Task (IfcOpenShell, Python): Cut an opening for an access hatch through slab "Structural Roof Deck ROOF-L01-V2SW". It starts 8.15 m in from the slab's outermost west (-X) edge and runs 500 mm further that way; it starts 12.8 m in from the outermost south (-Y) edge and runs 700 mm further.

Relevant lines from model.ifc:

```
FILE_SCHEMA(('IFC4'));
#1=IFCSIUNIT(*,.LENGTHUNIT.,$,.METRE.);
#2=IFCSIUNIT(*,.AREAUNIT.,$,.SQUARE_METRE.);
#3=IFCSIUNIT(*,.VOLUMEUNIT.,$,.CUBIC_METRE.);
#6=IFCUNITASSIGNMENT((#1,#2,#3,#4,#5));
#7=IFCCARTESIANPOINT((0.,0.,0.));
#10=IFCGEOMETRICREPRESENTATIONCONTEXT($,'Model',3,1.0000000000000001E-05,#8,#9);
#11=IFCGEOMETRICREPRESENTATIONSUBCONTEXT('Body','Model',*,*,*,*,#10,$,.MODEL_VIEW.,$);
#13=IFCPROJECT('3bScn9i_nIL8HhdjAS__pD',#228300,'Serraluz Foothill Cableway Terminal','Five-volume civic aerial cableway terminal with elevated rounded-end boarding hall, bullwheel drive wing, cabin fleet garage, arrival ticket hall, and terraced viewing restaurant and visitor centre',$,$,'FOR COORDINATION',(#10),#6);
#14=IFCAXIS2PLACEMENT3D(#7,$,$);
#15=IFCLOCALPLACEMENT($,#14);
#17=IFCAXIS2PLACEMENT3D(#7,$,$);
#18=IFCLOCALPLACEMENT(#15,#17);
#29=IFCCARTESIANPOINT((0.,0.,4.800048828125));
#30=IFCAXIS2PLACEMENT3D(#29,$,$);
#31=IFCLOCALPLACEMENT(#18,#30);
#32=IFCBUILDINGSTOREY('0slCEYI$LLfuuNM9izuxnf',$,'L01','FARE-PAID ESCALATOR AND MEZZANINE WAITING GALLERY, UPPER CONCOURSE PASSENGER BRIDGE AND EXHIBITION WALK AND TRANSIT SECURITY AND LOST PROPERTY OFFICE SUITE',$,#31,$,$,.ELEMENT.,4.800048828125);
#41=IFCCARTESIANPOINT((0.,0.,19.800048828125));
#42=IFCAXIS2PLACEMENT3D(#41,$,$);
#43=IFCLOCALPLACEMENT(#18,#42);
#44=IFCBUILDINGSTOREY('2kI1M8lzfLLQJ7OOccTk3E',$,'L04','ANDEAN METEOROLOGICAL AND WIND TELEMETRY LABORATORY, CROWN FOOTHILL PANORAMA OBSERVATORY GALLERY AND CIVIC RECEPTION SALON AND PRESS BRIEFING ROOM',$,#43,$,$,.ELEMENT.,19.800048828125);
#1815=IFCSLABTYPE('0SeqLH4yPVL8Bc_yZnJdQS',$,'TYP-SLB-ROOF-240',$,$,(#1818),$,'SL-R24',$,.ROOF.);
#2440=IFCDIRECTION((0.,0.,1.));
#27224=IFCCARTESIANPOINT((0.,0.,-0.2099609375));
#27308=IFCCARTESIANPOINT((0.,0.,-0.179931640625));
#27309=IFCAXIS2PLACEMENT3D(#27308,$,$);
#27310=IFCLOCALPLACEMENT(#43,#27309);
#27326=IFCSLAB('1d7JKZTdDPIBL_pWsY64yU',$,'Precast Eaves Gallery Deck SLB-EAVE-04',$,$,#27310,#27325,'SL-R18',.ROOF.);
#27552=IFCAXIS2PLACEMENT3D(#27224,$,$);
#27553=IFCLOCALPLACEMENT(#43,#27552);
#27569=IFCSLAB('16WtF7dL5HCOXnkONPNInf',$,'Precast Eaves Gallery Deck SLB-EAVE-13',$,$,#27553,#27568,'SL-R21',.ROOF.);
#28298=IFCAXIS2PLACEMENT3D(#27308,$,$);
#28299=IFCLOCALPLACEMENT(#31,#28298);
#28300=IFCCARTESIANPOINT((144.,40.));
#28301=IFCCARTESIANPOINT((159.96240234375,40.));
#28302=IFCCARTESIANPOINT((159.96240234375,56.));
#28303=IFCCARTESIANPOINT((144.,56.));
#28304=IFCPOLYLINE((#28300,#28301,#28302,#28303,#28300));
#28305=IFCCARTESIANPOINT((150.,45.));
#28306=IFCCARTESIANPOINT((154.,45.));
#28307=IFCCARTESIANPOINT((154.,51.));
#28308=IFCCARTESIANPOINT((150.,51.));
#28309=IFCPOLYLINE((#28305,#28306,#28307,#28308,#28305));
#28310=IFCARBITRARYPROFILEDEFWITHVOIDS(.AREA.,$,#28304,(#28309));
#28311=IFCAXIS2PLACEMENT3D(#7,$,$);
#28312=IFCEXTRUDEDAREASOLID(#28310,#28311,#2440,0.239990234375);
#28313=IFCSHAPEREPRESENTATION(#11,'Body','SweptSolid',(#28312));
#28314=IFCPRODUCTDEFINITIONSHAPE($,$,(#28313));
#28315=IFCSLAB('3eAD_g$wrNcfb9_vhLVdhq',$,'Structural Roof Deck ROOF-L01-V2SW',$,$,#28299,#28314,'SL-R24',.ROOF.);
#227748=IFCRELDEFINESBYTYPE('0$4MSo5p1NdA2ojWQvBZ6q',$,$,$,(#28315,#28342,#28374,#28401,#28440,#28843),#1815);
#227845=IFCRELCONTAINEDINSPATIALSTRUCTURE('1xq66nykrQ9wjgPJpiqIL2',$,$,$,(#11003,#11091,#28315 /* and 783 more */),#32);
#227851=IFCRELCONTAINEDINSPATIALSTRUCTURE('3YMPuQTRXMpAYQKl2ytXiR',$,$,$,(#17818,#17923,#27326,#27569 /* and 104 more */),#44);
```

```python
import numpy as np
import ifcopenshell
import ifcopenshell.api.feature
import ifcopenshell.api.geometry
import ifcopenshell.api.root
import ifcopenshell.geom
import ifcopenshell.util.placement
import ifcopenshell.util.representation
import ifcopenshell.util.shape
import ifcopenshell.util.unit

model = ifcopenshell.open("model.ifc")
unit_scale = ifcopenshell.util.unit.calculate_unit_scale(model)
settings = ifcopenshell.geom.settings()


def volume(element):
    """Net volume in cubic metres, openings subtracted."""
    shape = ifcopenshell.geom.create_shape(settings, element)
    return ifcopenshell.util.shape.get_volume(shape.geometry)


slab = model.by_guid("3eAD_g$wrNcfb9_vhLVdhq")
before = volume(slab)

# Extent in the slab's own axes, in metres. The edges named are its -X and -Y sides.
slab_shape = ifcopenshell.geom.create_shape(settings, slab)
vertices = ifcopenshell.util.shape.get_vertices(slab_shape.geometry)
x_min, y_min, bottom = vertices.min(axis=0)
top = vertices[:, 2].max()

opening = ifcopenshell.api.root.create_entity(model, ifc_class="IfcOpeningElement", name="Access hatch opening", predefined_type="OPENING")
context = ifcopenshell.util.representation.get_context(model, "Model", "Body", "MODEL_VIEW")
width, depth = 0.5, 0.7
outline = [(0.0, 0.0), (width, 0.0), (width, depth), (0.0, depth), (0.0, 0.0)]
# Overshoot both faces by 50 mm so the cut is clean.
shape = ifcopenshell.api.geometry.add_slab_representation(
    model, context=context, depth=top - bottom + 0.1, polyline=outline
)
ifcopenshell.api.geometry.assign_representation(model, product=opening, representation=shape)

matrix = ifcopenshell.util.placement.get_local_placement(slab.ObjectPlacement)
matrix[:, 3] = matrix @ np.append(np.array([x_min + 8.15, y_min + 12.8, bottom - 0.05]) / unit_scale, 1.0)
ifcopenshell.api.geometry.edit_object_placement(model, product=opening, matrix=matrix, is_si=False)
ifcopenshell.api.feature.add_feature(model, feature=opening, element=slab)

after = volume(slab)

print(f"slab volume {before:.3f} -> {after:.3f} m3")

model.write("model_rev.ifc")
```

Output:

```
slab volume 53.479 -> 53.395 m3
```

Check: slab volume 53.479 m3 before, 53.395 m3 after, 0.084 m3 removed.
